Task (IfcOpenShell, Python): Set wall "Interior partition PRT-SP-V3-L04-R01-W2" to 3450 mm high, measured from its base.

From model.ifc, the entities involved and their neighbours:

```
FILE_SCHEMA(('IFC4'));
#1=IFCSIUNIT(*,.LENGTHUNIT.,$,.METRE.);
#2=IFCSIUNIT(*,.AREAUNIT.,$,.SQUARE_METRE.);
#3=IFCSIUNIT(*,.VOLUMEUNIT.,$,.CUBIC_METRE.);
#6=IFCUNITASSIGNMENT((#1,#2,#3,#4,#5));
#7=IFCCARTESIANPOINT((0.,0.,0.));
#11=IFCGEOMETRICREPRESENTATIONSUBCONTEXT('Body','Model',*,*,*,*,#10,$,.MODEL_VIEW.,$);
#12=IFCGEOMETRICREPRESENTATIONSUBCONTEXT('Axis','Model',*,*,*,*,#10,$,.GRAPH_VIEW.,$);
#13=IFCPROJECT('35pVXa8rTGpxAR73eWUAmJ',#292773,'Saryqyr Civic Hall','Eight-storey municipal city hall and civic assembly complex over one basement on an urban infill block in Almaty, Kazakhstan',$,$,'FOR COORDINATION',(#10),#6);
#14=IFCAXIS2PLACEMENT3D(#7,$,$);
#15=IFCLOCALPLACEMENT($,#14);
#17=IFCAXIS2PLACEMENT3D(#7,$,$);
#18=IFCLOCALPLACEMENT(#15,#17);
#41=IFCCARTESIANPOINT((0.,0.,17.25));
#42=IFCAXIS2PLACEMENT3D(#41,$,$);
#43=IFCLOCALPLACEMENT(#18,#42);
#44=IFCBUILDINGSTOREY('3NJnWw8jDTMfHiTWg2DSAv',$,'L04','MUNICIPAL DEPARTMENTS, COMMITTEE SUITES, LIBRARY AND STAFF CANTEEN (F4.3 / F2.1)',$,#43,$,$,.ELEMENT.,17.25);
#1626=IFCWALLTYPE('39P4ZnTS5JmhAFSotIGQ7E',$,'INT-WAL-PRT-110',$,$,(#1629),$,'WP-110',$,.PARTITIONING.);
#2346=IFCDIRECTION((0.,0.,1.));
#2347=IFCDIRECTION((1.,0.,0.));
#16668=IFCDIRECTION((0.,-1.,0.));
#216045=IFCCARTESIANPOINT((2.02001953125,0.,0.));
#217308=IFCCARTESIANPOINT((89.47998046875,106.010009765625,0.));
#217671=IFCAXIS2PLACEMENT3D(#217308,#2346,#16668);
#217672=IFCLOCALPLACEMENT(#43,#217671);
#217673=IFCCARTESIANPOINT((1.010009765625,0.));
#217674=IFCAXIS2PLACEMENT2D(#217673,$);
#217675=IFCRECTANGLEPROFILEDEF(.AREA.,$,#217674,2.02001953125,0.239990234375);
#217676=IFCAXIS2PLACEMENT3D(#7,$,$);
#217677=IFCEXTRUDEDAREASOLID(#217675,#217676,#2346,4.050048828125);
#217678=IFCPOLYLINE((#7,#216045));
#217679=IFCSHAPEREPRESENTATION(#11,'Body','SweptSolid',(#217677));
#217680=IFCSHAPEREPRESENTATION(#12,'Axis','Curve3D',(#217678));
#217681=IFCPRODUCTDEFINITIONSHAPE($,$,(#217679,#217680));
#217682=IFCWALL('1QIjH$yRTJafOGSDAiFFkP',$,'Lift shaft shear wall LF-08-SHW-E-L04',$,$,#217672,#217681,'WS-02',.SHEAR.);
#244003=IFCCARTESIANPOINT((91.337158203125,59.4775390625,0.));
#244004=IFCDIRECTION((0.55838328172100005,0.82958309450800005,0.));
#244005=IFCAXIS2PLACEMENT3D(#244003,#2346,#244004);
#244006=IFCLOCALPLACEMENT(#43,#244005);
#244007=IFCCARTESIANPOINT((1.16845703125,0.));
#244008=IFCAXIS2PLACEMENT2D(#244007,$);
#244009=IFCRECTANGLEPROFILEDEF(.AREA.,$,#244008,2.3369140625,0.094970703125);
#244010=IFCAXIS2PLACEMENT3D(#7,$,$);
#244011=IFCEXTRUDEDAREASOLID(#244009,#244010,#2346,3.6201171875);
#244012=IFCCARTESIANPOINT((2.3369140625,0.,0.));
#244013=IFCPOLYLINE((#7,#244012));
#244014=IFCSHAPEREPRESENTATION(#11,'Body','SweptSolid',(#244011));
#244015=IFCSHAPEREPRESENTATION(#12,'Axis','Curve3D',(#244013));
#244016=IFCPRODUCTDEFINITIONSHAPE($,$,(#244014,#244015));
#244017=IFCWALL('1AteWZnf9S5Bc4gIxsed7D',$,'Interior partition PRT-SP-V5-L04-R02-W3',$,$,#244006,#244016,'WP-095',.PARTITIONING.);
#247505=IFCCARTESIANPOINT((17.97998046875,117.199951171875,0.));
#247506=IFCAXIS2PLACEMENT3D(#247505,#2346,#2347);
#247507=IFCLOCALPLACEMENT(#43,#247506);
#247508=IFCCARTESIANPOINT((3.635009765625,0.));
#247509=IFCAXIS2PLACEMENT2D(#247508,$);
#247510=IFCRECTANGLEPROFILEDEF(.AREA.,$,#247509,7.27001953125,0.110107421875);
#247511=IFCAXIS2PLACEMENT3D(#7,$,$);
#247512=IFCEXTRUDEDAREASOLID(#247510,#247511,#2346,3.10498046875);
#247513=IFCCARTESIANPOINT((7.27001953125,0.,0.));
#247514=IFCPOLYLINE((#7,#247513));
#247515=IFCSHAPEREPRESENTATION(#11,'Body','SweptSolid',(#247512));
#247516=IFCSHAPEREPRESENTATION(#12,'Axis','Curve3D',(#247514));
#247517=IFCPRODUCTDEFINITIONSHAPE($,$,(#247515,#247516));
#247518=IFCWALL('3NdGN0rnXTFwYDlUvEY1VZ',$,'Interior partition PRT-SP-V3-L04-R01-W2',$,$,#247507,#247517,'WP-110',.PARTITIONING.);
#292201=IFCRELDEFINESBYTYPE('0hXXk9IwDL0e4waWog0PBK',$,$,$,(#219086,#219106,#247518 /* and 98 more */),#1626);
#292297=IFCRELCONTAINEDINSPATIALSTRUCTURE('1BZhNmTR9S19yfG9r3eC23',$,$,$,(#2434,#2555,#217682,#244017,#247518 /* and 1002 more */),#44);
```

```python
import ifcopenshell
import ifcopenshell.geom
import ifcopenshell.util.representation
import ifcopenshell.util.shape
import ifcopenshell.util.unit

model = ifcopenshell.open("model.ifc")
unit_scale = ifcopenshell.util.unit.calculate_unit_scale(model)
settings = ifcopenshell.geom.settings()


def volume(element):
    """Net volume in cubic metres, openings subtracted."""
    shape = ifcopenshell.geom.create_shape(settings, element)
    return ifcopenshell.util.shape.get_volume(shape.geometry)


wall = model.by_guid("3NdGN0rnXTFwYDlUvEY1VZ")
before = volume(wall)

body = ifcopenshell.util.representation.get_representation(wall, "Model", "Body")
solid = body.Items[0]
old_height = solid.Depth
solid.Depth = 3.45 / unit_scale
after = volume(wall)

print(f"height {old_height:g} -> {solid.Depth:g}, volume {before:.3f} -> {after:.3f} m3")

model.write("model-out.ifc")
```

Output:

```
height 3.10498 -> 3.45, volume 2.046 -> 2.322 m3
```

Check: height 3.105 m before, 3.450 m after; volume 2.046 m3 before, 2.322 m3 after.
